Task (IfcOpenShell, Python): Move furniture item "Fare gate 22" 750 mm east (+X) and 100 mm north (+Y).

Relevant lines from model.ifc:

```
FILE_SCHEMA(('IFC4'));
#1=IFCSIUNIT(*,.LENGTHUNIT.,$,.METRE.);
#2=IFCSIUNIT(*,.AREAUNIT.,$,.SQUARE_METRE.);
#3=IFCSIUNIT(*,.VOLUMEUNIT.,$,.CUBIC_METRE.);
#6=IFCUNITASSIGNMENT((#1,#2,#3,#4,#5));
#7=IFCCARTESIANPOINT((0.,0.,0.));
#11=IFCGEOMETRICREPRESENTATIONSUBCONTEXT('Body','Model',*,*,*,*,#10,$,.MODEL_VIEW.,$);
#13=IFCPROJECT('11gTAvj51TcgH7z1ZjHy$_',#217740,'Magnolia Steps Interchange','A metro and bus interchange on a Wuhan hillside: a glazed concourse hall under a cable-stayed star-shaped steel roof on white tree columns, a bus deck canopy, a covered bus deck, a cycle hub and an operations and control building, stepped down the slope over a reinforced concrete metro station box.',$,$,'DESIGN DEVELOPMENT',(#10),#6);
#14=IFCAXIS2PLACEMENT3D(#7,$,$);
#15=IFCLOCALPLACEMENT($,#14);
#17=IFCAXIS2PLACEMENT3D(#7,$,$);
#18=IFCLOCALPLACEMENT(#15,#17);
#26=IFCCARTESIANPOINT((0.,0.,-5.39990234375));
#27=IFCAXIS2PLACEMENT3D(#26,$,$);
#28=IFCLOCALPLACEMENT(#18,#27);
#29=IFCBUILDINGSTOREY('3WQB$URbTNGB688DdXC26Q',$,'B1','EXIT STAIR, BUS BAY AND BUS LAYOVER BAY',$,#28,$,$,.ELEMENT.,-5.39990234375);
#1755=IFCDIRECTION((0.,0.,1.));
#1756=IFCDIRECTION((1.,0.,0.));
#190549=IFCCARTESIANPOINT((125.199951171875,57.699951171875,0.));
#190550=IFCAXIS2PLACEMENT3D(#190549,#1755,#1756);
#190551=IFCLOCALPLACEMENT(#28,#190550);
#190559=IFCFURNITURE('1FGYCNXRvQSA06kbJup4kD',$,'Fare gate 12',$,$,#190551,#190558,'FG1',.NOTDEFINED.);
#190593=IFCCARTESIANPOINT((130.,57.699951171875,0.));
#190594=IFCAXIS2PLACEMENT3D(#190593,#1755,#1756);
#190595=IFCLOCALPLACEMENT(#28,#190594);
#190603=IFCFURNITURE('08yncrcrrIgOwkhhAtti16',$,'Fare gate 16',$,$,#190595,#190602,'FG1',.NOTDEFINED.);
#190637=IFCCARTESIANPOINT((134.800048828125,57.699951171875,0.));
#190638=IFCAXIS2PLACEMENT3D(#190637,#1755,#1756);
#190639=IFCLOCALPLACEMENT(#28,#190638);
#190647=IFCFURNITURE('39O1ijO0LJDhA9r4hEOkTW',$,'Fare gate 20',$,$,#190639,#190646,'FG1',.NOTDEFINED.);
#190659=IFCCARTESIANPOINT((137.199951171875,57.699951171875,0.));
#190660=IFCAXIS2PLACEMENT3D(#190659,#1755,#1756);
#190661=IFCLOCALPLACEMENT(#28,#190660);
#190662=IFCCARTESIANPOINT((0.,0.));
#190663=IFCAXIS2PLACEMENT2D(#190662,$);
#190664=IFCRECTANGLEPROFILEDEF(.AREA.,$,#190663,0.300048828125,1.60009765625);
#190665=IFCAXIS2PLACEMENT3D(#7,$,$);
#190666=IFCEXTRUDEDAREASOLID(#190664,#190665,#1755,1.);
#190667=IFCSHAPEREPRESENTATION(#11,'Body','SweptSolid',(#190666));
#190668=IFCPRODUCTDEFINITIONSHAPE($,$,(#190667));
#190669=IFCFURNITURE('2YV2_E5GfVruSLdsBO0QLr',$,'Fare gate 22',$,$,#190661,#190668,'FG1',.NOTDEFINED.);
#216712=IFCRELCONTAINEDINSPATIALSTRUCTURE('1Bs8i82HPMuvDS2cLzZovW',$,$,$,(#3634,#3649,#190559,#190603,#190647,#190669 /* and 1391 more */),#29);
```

```python
import ifcopenshell
import ifcopenshell.api.geometry
import ifcopenshell.util.placement
import ifcopenshell.util.unit

model = ifcopenshell.open("model.ifc")
unit_scale = ifcopenshell.util.unit.calculate_unit_scale(model)

item = model.by_guid("2YV2_E5GfVruSLdsBO0QLr")
matrix = ifcopenshell.util.placement.get_local_placement(item.ObjectPlacement)
matrix[0, 3] += 0.75 / unit_scale
matrix[1, 3] += 0.1 / unit_scale
ifcopenshell.api.geometry.edit_object_placement(model, product=item, matrix=matrix, is_si=False)

print(ifcopenshell.util.placement.get_local_placement(item.ObjectPlacement).round(3) + 0.0)

model.write("model_updated.ifc")
```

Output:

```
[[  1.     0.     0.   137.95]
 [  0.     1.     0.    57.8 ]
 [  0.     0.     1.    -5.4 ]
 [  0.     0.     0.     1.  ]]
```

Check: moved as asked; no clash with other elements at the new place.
